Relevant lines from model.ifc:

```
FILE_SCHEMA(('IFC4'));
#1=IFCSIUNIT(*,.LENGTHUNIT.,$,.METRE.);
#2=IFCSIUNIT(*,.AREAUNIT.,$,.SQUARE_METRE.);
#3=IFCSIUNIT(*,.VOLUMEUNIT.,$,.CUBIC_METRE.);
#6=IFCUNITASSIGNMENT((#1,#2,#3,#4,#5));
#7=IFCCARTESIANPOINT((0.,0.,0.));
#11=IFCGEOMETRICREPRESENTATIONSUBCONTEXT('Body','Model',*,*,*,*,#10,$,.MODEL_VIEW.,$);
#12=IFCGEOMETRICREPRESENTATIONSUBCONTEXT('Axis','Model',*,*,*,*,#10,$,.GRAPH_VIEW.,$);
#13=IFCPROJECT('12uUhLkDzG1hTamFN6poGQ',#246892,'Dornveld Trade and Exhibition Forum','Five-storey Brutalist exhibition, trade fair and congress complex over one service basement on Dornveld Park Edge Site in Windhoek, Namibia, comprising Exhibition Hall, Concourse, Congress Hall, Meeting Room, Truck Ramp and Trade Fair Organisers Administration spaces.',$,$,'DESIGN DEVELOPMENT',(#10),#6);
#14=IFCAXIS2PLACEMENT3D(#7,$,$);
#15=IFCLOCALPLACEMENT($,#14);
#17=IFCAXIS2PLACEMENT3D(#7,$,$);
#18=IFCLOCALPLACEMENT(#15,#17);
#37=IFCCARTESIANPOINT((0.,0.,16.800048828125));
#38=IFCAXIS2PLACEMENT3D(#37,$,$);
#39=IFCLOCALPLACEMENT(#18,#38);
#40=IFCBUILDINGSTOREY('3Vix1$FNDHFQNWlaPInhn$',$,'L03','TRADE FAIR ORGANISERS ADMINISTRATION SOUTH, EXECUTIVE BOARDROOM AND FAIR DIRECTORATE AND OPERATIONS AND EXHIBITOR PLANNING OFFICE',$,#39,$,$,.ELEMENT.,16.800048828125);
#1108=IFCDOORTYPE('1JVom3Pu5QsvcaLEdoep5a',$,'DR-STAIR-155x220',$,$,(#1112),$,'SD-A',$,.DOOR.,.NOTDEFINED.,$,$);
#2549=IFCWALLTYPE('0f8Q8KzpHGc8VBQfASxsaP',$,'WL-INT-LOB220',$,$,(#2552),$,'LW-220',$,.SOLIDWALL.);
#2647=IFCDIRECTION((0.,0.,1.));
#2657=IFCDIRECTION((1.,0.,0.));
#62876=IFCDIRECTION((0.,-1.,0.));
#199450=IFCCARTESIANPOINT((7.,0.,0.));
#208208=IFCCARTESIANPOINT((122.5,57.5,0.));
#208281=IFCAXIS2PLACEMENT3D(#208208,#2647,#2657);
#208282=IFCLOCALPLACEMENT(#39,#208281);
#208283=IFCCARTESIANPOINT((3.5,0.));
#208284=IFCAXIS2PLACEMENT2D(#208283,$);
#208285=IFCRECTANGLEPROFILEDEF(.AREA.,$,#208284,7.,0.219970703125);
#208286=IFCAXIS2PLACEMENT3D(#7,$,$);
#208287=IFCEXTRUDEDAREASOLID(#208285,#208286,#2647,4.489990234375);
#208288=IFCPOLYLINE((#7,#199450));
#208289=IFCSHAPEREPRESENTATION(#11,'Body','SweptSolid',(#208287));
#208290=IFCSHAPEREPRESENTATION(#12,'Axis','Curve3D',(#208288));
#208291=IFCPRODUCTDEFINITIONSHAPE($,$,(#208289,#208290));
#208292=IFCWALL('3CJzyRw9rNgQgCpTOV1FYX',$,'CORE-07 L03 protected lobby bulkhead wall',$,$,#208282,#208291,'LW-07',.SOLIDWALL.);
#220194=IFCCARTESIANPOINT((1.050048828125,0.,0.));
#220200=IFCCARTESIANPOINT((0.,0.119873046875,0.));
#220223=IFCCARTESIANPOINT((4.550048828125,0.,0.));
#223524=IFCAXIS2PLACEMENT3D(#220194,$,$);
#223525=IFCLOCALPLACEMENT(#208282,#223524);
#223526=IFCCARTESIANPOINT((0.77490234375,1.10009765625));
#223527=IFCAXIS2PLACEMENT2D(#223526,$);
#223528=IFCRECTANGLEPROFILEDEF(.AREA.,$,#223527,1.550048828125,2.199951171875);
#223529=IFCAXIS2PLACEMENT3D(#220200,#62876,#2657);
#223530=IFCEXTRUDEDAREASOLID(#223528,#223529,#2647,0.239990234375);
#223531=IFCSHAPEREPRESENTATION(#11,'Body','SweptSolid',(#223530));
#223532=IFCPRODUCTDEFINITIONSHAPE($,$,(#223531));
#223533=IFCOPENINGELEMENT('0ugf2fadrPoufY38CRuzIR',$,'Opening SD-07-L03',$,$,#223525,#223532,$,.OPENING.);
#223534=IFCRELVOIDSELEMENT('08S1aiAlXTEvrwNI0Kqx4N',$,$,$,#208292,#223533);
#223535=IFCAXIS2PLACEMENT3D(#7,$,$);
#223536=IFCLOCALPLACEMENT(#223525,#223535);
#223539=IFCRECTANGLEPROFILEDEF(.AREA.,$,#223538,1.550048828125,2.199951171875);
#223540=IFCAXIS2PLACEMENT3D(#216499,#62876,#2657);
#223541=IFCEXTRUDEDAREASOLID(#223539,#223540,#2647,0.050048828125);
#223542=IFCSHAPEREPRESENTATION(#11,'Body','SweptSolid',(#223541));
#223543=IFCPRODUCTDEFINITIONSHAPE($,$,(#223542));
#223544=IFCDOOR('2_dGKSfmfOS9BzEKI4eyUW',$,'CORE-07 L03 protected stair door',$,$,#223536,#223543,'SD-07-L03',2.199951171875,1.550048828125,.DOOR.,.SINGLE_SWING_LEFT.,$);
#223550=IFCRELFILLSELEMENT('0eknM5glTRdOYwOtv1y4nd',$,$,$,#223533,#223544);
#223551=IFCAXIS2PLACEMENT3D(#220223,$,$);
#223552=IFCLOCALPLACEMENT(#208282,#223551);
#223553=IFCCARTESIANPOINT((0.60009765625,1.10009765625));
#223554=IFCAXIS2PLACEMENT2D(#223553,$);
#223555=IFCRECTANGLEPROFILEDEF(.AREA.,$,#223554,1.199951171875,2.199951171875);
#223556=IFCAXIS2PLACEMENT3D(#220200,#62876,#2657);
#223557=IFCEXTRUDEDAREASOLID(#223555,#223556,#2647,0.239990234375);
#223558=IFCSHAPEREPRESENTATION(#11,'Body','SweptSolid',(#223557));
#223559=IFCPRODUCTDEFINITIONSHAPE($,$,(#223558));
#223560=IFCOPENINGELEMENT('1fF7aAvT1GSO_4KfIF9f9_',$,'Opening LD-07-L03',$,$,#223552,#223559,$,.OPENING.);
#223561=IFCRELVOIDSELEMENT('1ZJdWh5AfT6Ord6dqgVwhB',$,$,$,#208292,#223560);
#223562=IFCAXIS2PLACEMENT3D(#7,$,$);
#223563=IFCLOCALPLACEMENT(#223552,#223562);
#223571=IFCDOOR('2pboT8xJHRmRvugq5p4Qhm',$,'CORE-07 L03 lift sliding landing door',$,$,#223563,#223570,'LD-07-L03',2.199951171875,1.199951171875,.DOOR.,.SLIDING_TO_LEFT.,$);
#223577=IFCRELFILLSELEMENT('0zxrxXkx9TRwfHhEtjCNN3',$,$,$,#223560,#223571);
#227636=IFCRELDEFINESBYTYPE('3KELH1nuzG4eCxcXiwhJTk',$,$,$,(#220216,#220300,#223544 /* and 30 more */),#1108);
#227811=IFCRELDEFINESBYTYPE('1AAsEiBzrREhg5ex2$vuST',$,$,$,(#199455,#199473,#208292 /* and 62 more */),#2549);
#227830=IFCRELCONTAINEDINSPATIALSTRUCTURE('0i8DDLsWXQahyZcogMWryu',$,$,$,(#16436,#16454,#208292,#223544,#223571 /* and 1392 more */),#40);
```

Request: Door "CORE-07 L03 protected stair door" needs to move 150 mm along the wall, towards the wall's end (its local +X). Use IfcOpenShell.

```python
import ifcopenshell
import ifcopenshell.api.geometry
import ifcopenshell.util.placement
import ifcopenshell.util.unit

model = ifcopenshell.open("model.ifc")
unit_scale = ifcopenshell.util.unit.calculate_unit_scale(model)

door = model.by_guid("2_dGKSfmfOS9BzEKI4eyUW")
opening = door.FillsVoids[0].RelatingOpeningElement
wall = opening.VoidsElements[0].RelatingBuildingElement

wall_matrix = ifcopenshell.util.placement.get_local_placement(wall.ObjectPlacement)
shift = wall_matrix[:3, 0] * 0.15 / unit_scale
before = ifcopenshell.util.placement.get_local_placement(door.ObjectPlacement)[:3, 3].copy()

# The door is placed relative to its opening, so it follows when the opening moves.
matrix = ifcopenshell.util.placement.get_local_placement(opening.ObjectPlacement)
matrix[:3, 3] += shift
ifcopenshell.api.geometry.edit_object_placement(
    model, product=opening, matrix=matrix, is_si=False, should_transform_children=True
)

after = ifcopenshell.util.placement.get_local_placement(door.ObjectPlacement)[:3, 3]
print("door moved by", (after - before).round(3) + 0.0)

model.write("model-out.ifc")
```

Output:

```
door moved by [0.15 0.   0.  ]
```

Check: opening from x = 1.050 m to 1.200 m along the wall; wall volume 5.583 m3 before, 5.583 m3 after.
